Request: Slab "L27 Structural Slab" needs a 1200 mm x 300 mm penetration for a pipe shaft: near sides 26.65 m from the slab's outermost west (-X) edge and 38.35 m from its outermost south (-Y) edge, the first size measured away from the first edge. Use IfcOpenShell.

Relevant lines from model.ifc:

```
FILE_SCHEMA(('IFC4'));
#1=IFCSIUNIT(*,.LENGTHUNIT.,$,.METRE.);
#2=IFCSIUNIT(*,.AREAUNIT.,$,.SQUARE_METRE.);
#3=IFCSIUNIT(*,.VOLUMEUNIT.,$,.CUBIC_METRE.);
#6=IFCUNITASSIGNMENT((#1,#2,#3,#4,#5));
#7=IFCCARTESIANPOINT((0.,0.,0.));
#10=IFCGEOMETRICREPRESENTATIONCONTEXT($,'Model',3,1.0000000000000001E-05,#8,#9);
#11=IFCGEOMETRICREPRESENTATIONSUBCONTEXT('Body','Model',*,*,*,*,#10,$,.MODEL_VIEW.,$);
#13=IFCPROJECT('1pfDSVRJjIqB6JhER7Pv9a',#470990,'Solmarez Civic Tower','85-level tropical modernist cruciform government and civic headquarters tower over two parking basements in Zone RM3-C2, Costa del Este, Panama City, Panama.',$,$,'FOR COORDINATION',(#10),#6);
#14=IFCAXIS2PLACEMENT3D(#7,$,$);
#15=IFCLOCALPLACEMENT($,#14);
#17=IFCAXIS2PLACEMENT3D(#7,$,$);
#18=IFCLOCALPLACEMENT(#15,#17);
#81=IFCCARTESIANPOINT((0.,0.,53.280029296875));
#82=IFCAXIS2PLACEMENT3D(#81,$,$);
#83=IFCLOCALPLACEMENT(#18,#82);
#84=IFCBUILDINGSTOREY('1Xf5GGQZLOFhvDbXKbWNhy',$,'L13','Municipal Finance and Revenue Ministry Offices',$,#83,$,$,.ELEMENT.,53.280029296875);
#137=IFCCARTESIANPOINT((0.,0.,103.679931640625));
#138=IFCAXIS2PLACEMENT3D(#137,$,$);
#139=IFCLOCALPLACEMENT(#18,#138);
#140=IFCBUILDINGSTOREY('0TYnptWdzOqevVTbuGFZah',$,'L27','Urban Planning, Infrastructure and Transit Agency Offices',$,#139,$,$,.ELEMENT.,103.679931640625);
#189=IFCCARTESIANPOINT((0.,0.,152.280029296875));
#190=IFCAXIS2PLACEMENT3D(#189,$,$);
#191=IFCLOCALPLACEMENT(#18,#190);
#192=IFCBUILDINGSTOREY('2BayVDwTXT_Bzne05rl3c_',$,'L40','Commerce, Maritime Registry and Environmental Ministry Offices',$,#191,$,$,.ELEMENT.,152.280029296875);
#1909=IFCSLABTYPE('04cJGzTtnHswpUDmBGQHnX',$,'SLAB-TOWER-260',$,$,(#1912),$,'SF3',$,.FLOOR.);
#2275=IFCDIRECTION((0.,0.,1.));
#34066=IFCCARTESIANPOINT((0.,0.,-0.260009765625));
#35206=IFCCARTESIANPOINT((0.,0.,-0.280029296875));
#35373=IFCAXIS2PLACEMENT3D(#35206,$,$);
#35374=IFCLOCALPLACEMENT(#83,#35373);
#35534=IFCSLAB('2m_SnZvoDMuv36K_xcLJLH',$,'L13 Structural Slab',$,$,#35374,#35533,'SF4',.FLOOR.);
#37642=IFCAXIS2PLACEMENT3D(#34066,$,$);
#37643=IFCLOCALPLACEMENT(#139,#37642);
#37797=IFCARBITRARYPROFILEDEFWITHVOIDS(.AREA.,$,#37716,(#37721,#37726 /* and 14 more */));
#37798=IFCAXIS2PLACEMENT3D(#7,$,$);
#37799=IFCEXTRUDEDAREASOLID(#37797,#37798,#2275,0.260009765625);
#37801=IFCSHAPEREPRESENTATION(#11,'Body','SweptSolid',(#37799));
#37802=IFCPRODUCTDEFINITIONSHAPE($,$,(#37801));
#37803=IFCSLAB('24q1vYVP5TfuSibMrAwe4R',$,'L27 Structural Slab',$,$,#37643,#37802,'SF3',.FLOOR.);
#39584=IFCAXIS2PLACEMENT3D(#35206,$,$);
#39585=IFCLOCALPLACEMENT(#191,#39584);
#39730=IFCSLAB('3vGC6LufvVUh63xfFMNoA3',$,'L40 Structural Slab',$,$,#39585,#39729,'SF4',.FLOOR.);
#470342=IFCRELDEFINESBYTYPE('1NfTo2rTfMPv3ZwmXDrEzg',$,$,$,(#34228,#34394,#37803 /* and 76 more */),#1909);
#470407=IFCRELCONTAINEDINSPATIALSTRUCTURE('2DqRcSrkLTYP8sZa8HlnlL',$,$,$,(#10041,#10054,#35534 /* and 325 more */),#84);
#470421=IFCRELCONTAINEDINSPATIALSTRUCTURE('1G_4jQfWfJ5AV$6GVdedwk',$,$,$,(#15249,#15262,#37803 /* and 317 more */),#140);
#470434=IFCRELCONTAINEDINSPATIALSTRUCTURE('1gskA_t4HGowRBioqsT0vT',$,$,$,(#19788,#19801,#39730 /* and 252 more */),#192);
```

```python
import numpy as np
import ifcopenshell
import ifcopenshell.api.feature
import ifcopenshell.api.geometry
import ifcopenshell.api.root
import ifcopenshell.geom
import ifcopenshell.util.placement
import ifcopenshell.util.representation
import ifcopenshell.util.shape
import ifcopenshell.util.unit

model = ifcopenshell.open("model.ifc")
unit_scale = ifcopenshell.util.unit.calculate_unit_scale(model)
settings = ifcopenshell.geom.settings()


def volume(element):
    """Net volume in cubic metres, openings subtracted."""
    shape = ifcopenshell.geom.create_shape(settings, element)
    return ifcopenshell.util.shape.get_volume(shape.geometry)


slab = model.by_guid("24q1vYVP5TfuSibMrAwe4R")
before = volume(slab)

# Extent in the slab's own axes, in metres. The edges named are its -X and -Y sides.
slab_shape = ifcopenshell.geom.create_shape(settings, slab)
vertices = ifcopenshell.util.shape.get_vertices(slab_shape.geometry)
x_min, y_min, bottom = vertices.min(axis=0)
top = vertices[:, 2].max()

opening = ifcopenshell.api.root.create_entity(model, ifc_class="IfcOpeningElement", name="Pipe shaft opening", predefined_type="OPENING")
context = ifcopenshell.util.representation.get_context(model, "Model", "Body", "MODEL_VIEW")
width, depth = 1.2, 0.3
outline = [(0.0, 0.0), (width, 0.0), (width, depth), (0.0, depth), (0.0, 0.0)]
# Overshoot both faces by 50 mm so the cut is clean.
shape = ifcopenshell.api.geometry.add_slab_representation(
    model, context=context, depth=top - bottom + 0.1, polyline=outline
)
ifcopenshell.api.geometry.assign_representation(model, product=opening, representation=shape)

matrix = ifcopenshell.util.placement.get_local_placement(slab.ObjectPlacement)
matrix[:, 3] = matrix @ np.append(np.array([x_min + 26.65, y_min + 38.35, bottom - 0.05]) / unit_scale, 1.0)
ifcopenshell.api.geometry.edit_object_placement(model, product=opening, matrix=matrix, is_si=False)
ifcopenshell.api.feature.add_feature(model, feature=opening, element=slab)

after = volume(slab)

print(f"slab volume {before:.3f} -> {after:.3f} m3")

model.write("model_updated.ifc")
```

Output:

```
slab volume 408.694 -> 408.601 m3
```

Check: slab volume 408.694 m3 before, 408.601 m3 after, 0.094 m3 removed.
